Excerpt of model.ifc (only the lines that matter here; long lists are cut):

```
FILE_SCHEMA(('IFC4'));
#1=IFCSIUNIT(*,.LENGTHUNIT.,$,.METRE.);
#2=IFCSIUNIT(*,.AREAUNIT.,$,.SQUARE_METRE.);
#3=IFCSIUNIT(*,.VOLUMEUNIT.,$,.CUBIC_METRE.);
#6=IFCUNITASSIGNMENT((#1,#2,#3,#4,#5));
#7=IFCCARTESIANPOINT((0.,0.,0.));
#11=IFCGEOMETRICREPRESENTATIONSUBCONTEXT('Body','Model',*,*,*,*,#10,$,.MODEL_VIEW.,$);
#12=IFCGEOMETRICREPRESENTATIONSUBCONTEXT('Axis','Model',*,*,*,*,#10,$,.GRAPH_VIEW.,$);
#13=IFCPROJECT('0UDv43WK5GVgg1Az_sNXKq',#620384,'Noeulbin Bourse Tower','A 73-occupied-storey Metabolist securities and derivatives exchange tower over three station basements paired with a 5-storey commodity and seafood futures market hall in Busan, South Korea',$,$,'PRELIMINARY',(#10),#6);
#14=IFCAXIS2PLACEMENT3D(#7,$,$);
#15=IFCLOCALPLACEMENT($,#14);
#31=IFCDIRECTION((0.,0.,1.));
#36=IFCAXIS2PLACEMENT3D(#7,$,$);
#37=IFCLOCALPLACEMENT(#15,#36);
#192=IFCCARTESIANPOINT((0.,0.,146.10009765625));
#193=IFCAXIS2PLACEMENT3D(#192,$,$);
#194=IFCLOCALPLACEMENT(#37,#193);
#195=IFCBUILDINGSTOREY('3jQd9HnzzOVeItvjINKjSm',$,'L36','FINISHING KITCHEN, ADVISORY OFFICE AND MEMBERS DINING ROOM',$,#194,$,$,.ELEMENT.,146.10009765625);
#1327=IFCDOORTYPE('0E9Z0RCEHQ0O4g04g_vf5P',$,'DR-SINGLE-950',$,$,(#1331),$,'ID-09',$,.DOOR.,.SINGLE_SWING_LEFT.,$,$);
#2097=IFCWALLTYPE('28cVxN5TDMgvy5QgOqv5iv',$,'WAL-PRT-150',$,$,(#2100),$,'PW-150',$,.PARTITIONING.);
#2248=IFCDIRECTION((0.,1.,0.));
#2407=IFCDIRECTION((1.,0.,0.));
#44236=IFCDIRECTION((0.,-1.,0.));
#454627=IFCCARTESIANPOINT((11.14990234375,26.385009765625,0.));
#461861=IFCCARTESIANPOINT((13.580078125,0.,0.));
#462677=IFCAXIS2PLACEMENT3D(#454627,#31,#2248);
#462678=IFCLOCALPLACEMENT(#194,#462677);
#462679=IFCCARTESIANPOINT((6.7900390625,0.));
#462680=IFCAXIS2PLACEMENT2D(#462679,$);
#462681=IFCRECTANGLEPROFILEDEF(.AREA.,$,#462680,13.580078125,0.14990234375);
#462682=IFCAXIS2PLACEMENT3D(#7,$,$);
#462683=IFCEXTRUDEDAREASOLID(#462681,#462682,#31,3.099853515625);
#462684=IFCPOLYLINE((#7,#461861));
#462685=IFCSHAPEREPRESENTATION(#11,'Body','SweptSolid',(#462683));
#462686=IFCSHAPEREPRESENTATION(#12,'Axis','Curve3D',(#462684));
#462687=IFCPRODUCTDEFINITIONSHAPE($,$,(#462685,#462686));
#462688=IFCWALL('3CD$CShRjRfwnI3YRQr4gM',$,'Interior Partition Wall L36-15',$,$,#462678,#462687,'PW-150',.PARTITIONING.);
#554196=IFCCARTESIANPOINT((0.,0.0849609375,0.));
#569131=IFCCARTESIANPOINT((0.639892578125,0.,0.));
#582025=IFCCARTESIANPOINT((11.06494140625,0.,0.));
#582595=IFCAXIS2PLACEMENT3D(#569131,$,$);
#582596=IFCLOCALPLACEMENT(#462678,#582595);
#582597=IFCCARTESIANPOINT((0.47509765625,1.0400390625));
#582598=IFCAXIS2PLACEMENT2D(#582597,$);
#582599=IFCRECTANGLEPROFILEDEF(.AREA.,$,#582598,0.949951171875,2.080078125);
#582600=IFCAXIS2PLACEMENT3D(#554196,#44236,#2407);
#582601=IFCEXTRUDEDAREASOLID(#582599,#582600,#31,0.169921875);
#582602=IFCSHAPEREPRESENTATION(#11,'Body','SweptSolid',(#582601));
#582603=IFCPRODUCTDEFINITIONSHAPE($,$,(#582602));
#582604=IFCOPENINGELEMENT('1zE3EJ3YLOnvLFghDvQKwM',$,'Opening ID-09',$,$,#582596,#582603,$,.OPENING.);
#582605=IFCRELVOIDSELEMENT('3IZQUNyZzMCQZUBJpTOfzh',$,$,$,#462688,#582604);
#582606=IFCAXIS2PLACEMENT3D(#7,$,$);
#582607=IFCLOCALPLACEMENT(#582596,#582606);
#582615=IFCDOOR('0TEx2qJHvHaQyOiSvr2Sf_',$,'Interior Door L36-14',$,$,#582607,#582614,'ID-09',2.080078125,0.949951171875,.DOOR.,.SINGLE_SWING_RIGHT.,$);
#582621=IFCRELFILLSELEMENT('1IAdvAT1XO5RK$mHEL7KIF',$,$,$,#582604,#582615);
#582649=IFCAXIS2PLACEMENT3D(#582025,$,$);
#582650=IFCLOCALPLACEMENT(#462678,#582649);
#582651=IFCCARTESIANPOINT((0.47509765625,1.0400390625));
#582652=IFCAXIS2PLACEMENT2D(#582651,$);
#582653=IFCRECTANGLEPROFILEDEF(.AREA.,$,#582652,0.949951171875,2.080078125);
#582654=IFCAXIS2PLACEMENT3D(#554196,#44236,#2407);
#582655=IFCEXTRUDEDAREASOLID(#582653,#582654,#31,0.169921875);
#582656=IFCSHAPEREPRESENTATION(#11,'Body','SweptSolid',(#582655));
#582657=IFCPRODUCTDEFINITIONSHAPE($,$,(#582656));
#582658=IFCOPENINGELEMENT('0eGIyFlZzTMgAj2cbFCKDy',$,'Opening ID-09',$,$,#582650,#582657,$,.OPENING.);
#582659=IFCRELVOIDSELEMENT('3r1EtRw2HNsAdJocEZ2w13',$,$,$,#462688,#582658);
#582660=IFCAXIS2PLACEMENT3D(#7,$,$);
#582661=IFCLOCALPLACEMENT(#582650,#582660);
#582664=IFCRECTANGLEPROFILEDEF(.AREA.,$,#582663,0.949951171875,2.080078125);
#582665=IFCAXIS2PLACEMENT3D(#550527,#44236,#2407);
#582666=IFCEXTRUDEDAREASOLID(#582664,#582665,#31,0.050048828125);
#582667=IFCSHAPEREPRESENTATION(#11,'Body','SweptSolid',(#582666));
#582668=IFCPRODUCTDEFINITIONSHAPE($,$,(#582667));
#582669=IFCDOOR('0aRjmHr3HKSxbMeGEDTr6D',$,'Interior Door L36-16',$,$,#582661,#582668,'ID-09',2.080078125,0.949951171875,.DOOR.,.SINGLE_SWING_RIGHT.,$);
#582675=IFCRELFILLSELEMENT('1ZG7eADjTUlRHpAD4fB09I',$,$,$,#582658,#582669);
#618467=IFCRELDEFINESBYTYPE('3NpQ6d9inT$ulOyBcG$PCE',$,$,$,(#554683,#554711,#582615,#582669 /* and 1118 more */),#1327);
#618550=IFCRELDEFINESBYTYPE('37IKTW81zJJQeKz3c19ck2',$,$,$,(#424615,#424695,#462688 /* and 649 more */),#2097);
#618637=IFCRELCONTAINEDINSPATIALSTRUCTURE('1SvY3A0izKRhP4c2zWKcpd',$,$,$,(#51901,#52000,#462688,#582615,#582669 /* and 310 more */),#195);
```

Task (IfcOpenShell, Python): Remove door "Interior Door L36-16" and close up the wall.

```python
import ifcopenshell
import ifcopenshell.api.feature
import ifcopenshell.api.root
import ifcopenshell.geom
import ifcopenshell.util.shape

model = ifcopenshell.open("model.ifc")
settings = ifcopenshell.geom.settings()


def volume(element):
    """Net volume in cubic metres, openings subtracted."""
    shape = ifcopenshell.geom.create_shape(settings, element)
    return ifcopenshell.util.shape.get_volume(shape.geometry)


door = model.by_guid("0aRjmHr3HKSxbMeGEDTr6D")
opening = door.FillsVoids[0].RelatingOpeningElement
wall = opening.VoidsElements[0].RelatingBuildingElement
before = volume(wall)

ifcopenshell.api.root.remove_product(model, product=door)
ifcopenshell.api.feature.remove_feature(model, feature=opening)

after = volume(wall)

print(f"wall volume {before:.3f} -> {after:.3f} m3")

model.write("model_edited.ifc")
```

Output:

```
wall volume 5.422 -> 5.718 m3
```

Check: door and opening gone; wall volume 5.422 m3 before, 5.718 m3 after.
